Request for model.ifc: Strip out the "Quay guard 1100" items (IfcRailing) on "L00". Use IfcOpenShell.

First a look at what the model holds.

```python
import ifcopenshell
import ifcopenshell.util.element

model = ifcopenshell.open("model.ifc")
print(model.schema)
storey = next(s for s in model.by_type("IfcBuildingStorey") if s.Name == "L00")
railings = [e for e in ifcopenshell.util.element.get_decomposition(storey) if e.is_a("IfcRailing")]
seen = {}
for e in railings:
    element_type = ifcopenshell.util.element.get_type(e)
    name = element_type.Name if element_type not in (None, e) else None
    seen[name] = seen.get(name, 0) + 1
for name, count in sorted(seen.items(), key=str):
    print(count, "x", name)
```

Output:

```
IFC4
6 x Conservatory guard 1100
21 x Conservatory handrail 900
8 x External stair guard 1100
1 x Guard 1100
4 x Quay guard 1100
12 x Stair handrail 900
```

```python
import ifcopenshell
import ifcopenshell.api.root
import ifcopenshell.util.element

model = ifcopenshell.open("model.ifc")

storey = next(s for s in model.by_type("IfcBuildingStorey") if s.Name == "L00")
railings = [e for e in ifcopenshell.util.element.get_decomposition(storey) if e.is_a("IfcRailing")]
targets = [e for e in railings if (t := ifcopenshell.util.element.get_type(e)) not in (None, e) and t.Name == "Quay guard 1100"]

for e in targets:
    ifcopenshell.api.root.remove_product(model, product=e)
print(len(targets), "removed")

model.write("model_rev.ifc")
```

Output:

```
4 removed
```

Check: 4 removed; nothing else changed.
